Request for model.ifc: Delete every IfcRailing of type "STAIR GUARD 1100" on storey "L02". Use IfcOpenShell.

First a look at what the model holds.

```python
import ifcopenshell
import ifcopenshell.util.element

model = ifcopenshell.open("model.ifc")
print(model.schema)
storey = next(s for s in model.by_type("IfcBuildingStorey") if s.Name == "L02")
railings = [e for e in ifcopenshell.util.element.get_decomposition(storey) if e.is_a("IfcRailing")]
seen = {}
for e in railings:
    element_type = ifcopenshell.util.element.get_type(e)
    name = element_type.Name if element_type not in (None, e) else None
    seen[name] = seen.get(name, 0) + 1
for name, count in sorted(seen.items(), key=str):
    print(count, "x", name)
```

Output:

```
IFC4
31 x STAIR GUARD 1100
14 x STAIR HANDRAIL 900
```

```python
import ifcopenshell
import ifcopenshell.api.root
import ifcopenshell.util.element

model = ifcopenshell.open("model.ifc")

storey = next(s for s in model.by_type("IfcBuildingStorey") if s.Name == "L02")
railings = [e for e in ifcopenshell.util.element.get_decomposition(storey) if e.is_a("IfcRailing")]
targets = [e for e in railings if (t := ifcopenshell.util.element.get_type(e)) not in (None, e) and t.Name == "STAIR GUARD 1100"]

for e in targets:
    ifcopenshell.api.root.remove_product(model, product=e)
print(len(targets), "removed")

model.write("model-out.ifc")
```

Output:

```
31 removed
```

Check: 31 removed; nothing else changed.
